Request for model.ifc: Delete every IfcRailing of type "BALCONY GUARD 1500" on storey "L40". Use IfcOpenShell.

First a look at what the model holds.

```python
import ifcopenshell
import ifcopenshell.util.element

model = ifcopenshell.open("model.ifc")
print(model.schema)
storey = next(s for s in model.by_type("IfcBuildingStorey") if s.Name == "L40")
railings = [e for e in ifcopenshell.util.element.get_decomposition(storey) if e.is_a("IfcRailing")]
seen = {}
for e in railings:
    element_type = ifcopenshell.util.element.get_type(e)
    name = element_type.Name if element_type not in (None, e) else None
    seen[name] = seen.get(name, 0) + 1
for name, count in sorted(seen.items(), key=str):
    print(count, "x", name)
```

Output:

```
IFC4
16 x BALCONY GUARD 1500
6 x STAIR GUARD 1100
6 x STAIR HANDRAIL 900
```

```python
import ifcopenshell
import ifcopenshell.api.root
import ifcopenshell.util.element

model = ifcopenshell.open("model.ifc")

storey = next(s for s in model.by_type("IfcBuildingStorey") if s.Name == "L40")
railings = [e for e in ifcopenshell.util.element.get_decomposition(storey) if e.is_a("IfcRailing")]
targets = [e for e in railings if (t := ifcopenshell.util.element.get_type(e)) not in (None, e) and t.Name == "BALCONY GUARD 1500"]

for e in targets:
    ifcopenshell.api.root.remove_product(model, product=e)
print(len(targets), "removed")

model.write("model_edited.ifc")
```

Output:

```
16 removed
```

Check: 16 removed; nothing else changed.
